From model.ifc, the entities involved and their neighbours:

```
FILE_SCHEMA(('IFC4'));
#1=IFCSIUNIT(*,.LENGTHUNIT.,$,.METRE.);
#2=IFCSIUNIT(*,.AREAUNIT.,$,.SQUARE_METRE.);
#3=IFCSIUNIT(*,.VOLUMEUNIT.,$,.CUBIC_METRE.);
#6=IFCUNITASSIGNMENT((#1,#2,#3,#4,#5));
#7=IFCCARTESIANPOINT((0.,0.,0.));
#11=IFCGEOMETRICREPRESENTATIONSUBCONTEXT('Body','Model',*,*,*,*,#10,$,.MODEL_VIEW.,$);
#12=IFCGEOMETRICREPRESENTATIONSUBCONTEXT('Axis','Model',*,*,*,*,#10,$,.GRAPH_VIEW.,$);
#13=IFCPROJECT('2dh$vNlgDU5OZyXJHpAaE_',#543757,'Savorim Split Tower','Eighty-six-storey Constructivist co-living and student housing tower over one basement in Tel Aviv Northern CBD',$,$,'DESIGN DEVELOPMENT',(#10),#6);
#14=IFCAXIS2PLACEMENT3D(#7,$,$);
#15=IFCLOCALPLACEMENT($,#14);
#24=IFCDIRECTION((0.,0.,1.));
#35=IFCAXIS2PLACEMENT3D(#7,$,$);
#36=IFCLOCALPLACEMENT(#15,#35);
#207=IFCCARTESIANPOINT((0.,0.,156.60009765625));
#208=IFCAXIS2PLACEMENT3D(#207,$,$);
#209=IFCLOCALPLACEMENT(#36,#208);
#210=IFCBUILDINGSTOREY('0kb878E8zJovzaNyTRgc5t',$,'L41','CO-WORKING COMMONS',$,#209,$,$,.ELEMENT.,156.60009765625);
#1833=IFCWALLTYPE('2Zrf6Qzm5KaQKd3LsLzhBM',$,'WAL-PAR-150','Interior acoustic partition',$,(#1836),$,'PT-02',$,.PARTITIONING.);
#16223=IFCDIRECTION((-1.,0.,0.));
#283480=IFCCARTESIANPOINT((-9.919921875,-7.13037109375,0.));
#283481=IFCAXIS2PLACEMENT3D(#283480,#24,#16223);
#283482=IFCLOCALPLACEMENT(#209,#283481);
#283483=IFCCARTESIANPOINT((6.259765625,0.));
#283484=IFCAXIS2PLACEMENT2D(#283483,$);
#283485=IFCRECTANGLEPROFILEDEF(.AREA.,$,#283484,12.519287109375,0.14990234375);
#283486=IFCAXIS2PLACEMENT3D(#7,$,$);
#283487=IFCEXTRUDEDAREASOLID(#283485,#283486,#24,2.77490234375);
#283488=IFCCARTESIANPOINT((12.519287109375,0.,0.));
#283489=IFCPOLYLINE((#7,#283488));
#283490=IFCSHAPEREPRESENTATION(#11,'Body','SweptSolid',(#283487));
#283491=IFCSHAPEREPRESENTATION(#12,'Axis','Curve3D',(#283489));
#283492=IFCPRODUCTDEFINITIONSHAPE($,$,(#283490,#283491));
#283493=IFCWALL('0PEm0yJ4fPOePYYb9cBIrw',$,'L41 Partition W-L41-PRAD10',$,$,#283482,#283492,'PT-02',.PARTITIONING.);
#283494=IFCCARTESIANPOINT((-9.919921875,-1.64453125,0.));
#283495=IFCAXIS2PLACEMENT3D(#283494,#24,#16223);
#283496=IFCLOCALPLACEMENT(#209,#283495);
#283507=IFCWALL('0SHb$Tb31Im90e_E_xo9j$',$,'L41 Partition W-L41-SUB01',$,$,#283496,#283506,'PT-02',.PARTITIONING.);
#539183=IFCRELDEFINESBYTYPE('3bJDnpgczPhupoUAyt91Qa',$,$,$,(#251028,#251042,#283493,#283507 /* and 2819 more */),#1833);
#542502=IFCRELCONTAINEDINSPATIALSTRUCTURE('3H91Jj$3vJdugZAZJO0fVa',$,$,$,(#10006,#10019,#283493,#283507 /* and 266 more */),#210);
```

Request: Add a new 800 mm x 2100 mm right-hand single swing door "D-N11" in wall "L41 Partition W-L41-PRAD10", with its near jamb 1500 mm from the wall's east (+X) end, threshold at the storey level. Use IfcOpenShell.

```python
import numpy as np
import ifcopenshell
import ifcopenshell.api.feature
import ifcopenshell.api.geometry
import ifcopenshell.api.root
import ifcopenshell.api.spatial
import ifcopenshell.geom
import ifcopenshell.util.element
import ifcopenshell.util.placement
import ifcopenshell.util.representation
import ifcopenshell.util.shape
import ifcopenshell.util.unit

model = ifcopenshell.open("model.ifc")
unit_scale = ifcopenshell.util.unit.calculate_unit_scale(model)
settings = ifcopenshell.geom.settings()


def volume(element):
    """Net volume in cubic metres, openings subtracted."""
    shape = ifcopenshell.geom.create_shape(settings, element)
    return ifcopenshell.util.shape.get_volume(shape.geometry)


wall = model.by_id(283493)
storey = ifcopenshell.util.element.get_container(wall, ifc_class="IfcBuildingStorey")
context = ifcopenshell.util.representation.get_context(model, "Model", "Body", "MODEL_VIEW")
before = volume(wall)

width, height, from_end, sill = 0.8, 2.1, 1.5, 0.0  # metres

# The wall runs along its own X axis, and the end named is its -X end.
wall_shape = ifcopenshell.geom.create_shape(settings, wall)
x, y, z = ifcopenshell.util.shape.get_vertices(wall_shape.geometry).T
start = x.min() + from_end
face, thickness = float(y.min()), float(y.max() - y.min())
wall_matrix = ifcopenshell.util.placement.get_local_placement(wall.ObjectPlacement)
level = ifcopenshell.util.placement.get_local_placement(storey.ObjectPlacement)[2, 3]


def in_wall(x, y):
    """Placement at x, y metres in the wall's axes, at sill height."""
    matrix = wall_matrix.copy()
    matrix[:, 3] = wall_matrix @ np.array([x / unit_scale, y / unit_scale, 0.0, 1.0])
    matrix[2, 3] = level + sill / unit_scale
    return matrix


# Opening: a box that overshoots both wall faces by 50 mm.
opening = ifcopenshell.api.root.create_entity(model, ifc_class="IfcOpeningElement", predefined_type="OPENING")
box = ifcopenshell.api.geometry.add_wall_representation(
    model, context=context, length=width, height=height, thickness=thickness + 0.1
)
ifcopenshell.api.geometry.assign_representation(model, product=opening, representation=box)
ifcopenshell.api.geometry.edit_object_placement(model, product=opening, matrix=in_wall(start, face - 0.05), is_si=False)
ifcopenshell.api.feature.add_feature(model, feature=opening, element=wall)

door = ifcopenshell.api.root.create_entity(model, ifc_class="IfcDoor", name="D-N11", predefined_type="DOOR")
door.OverallWidth, door.OverallHeight = width / unit_scale, height / unit_scale
door.OperationType = "SINGLE_SWING_RIGHT"
body = ifcopenshell.api.geometry.add_door_representation(
    model,
    context=context,
    overall_width=door.OverallWidth,
    overall_height=door.OverallHeight,
    operation_type="SINGLE_SWING_RIGHT",
    lining_properties={"LiningDepth": thickness / unit_scale, "ThresholdDepth": thickness / unit_scale},
)
ifcopenshell.api.geometry.assign_representation(model, product=door, representation=body)
ifcopenshell.api.spatial.assign_container(model, products=[door], relating_structure=storey)
ifcopenshell.api.feature.add_filling(model, opening=opening, element=door)

# The lining spans the wall, so the door starts at the wall face.
ifcopenshell.api.geometry.edit_object_placement(model, product=door, matrix=in_wall(start, face), is_si=False)

after = volume(wall)

print(f"wall volume {before:.3f} -> {after:.3f} m3")

model.write("model-out.ifc")
```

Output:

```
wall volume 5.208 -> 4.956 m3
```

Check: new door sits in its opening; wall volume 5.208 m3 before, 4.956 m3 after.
